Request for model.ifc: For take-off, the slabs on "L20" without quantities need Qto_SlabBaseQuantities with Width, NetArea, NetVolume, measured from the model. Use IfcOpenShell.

First a look at what the model holds.

```python
import ifcopenshell
import ifcopenshell.util.element
import ifcopenshell.util.unit

model = ifcopenshell.open("model.ifc")
print(model.schema)
for unit_type in ("LENGTHUNIT", "AREAUNIT", "VOLUMEUNIT"):
    print(unit_type, ifcopenshell.util.unit.calculate_unit_scale(model, unit_type))
storey = next(s for s in model.by_type("IfcBuildingStorey") if s.Name == "L20")
slabs = [e for e in ifcopenshell.util.element.get_decomposition(storey) if e.is_a("IfcSlab")]
for e in sorted(slabs, key=lambda e: e.id()):
    print(e.id(), e.is_a(), e.Name, list(ifcopenshell.util.element.get_psets(e, qtos_only=True)), sep=" | ")
```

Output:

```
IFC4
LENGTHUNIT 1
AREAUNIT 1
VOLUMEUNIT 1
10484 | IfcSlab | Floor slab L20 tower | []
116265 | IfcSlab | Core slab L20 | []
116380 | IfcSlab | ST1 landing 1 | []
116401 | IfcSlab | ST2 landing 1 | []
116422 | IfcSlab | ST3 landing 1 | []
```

```python
import ifcopenshell
import ifcopenshell.api.pset
import ifcopenshell.geom
import ifcopenshell.util.element
import ifcopenshell.util.shape
import ifcopenshell.util.unit

model = ifcopenshell.open("model.ifc")
unit_scale = ifcopenshell.util.unit.calculate_unit_scale(model)
area_scale = ifcopenshell.util.unit.calculate_unit_scale(model, "AREAUNIT")
volume_scale = ifcopenshell.util.unit.calculate_unit_scale(model, "VOLUMEUNIT")
settings = ifcopenshell.geom.settings()

storey = next(s for s in model.by_type("IfcBuildingStorey") if s.Name == "L20")
slabs = [e for e in ifcopenshell.util.element.get_decomposition(storey) if e.is_a("IfcSlab")]

for e in sorted(slabs, key=lambda e: e.id()):
    if ifcopenshell.util.element.get_psets(e, qtos_only=True, should_inherit=False):
        continue
    # Geometry comes back in metres, in the element's own axes.
    shape = ifcopenshell.geom.create_shape(settings, e)
    values = {
        "Width": ifcopenshell.util.shape.get_z(shape.geometry) / unit_scale,
        "NetArea": ifcopenshell.util.shape.get_footprint_area(shape.geometry) / area_scale,
        "NetVolume": ifcopenshell.util.shape.get_volume(shape.geometry) / volume_scale,
    }
    qto = ifcopenshell.api.pset.add_qto(model, product=e, name="Qto_SlabBaseQuantities")
    ifcopenshell.api.pset.edit_qto(model, qto=qto, properties=values)
    print(e.id(), {k: round(v, 3) for k, v in values.items()})

model.write("model_rev.ifc")
```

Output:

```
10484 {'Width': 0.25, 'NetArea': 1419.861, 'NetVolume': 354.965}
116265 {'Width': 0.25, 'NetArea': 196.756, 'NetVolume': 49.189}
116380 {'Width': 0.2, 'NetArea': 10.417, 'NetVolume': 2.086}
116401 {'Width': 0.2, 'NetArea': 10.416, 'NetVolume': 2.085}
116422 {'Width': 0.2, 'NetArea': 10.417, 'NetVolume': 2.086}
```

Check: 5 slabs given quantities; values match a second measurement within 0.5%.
